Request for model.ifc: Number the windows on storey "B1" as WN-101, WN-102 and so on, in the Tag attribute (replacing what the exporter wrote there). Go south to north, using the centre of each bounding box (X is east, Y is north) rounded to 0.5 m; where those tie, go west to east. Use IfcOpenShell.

First a look at what the model holds.

```python
import ifcopenshell
import ifcopenshell.util.element
import ifcopenshell.util.placement

model = ifcopenshell.open("model.ifc")
print(model.schema)
storey = next(s for s in model.by_type("IfcBuildingStorey") if s.Name == "B1")
windows = [e for e in ifcopenshell.util.element.get_decomposition(storey) if e.is_a("IfcWindow")]
for e in sorted(windows, key=lambda e: e.id()):
    origin = ifcopenshell.util.placement.get_local_placement(e.ObjectPlacement)[:3, 3]
    print(e.id(), e.Tag, e.Name, origin.round(2) + 0.0, sep=" | ")
```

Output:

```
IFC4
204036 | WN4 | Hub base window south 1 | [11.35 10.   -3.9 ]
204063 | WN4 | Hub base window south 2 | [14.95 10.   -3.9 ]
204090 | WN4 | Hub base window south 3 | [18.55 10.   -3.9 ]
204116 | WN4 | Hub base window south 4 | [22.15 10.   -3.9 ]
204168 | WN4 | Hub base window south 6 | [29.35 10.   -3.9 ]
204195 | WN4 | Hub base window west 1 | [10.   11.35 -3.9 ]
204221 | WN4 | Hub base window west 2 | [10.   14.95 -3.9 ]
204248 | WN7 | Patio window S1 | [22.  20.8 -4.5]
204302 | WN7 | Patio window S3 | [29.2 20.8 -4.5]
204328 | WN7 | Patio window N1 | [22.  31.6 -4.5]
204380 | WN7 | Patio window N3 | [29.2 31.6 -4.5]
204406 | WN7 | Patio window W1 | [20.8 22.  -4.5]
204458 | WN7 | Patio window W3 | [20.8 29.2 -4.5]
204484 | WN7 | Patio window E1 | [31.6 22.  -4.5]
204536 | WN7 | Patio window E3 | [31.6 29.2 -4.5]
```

```python
import ifcopenshell
import ifcopenshell.geom
import ifcopenshell.util.element
import ifcopenshell.util.shape

model = ifcopenshell.open("model.ifc")
settings = ifcopenshell.geom.settings()
settings.set("use-world-coords", True)


def centre(element):
    shape = ifcopenshell.geom.create_shape(settings, element)
    return ifcopenshell.util.shape.get_bbox_centroid(shape.geometry)


storey = next(s for s in model.by_type("IfcBuildingStorey") if s.Name == "B1")
windows = [e for e in ifcopenshell.util.element.get_decomposition(storey) if e.is_a("IfcWindow")]

# Insertion points can sit at a corner or the storey origin, so sort by the geometry (in metres).
centres = {e: centre(e) for e in windows}
windows.sort(key=lambda e: (round(centres[e][1] / 0.5), centres[e][0]))

for i, e in enumerate(windows, start=1):
    number = f"WN-1{i:02d}"
    e.Tag = number
    print(e.id(), number)

model.write("model_edited.ifc")
```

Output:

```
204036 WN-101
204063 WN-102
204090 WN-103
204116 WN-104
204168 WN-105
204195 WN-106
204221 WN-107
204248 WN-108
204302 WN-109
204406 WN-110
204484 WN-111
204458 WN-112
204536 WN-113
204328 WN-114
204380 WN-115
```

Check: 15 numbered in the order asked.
